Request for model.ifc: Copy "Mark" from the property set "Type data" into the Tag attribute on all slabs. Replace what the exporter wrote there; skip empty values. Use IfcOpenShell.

First a look at what the model holds.

```python
import ifcopenshell
import ifcopenshell.util.element

model = ifcopenshell.open("model.ifc")
print(model.schema)
slabs = model.by_type("IfcSlab")
print(len(slabs), "slabs")
for e in slabs[:8]:
    source = ifcopenshell.util.element.get_pset(e, "Type data", "Mark")
    target = e.Tag
    print(e.id(), repr(source), repr(target), sep=" | ")
```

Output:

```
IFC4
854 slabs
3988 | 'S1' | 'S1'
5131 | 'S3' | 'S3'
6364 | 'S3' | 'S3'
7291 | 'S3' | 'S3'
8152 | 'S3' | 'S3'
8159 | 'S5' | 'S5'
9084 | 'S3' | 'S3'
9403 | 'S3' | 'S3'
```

```python
import ifcopenshell
import ifcopenshell.util.element

model = ifcopenshell.open("model.ifc")

count = 0
for e in model.by_type("IfcSlab"):
    value = ifcopenshell.util.element.get_pset(e, "Type data", "Mark")
    current = e.Tag
    if not value or not value.strip() or current == value:
        continue
    e.Tag = value
    count += 1

print(count, "slabs updated")

model.write("model_edited.ifc")
```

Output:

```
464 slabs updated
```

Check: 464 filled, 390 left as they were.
